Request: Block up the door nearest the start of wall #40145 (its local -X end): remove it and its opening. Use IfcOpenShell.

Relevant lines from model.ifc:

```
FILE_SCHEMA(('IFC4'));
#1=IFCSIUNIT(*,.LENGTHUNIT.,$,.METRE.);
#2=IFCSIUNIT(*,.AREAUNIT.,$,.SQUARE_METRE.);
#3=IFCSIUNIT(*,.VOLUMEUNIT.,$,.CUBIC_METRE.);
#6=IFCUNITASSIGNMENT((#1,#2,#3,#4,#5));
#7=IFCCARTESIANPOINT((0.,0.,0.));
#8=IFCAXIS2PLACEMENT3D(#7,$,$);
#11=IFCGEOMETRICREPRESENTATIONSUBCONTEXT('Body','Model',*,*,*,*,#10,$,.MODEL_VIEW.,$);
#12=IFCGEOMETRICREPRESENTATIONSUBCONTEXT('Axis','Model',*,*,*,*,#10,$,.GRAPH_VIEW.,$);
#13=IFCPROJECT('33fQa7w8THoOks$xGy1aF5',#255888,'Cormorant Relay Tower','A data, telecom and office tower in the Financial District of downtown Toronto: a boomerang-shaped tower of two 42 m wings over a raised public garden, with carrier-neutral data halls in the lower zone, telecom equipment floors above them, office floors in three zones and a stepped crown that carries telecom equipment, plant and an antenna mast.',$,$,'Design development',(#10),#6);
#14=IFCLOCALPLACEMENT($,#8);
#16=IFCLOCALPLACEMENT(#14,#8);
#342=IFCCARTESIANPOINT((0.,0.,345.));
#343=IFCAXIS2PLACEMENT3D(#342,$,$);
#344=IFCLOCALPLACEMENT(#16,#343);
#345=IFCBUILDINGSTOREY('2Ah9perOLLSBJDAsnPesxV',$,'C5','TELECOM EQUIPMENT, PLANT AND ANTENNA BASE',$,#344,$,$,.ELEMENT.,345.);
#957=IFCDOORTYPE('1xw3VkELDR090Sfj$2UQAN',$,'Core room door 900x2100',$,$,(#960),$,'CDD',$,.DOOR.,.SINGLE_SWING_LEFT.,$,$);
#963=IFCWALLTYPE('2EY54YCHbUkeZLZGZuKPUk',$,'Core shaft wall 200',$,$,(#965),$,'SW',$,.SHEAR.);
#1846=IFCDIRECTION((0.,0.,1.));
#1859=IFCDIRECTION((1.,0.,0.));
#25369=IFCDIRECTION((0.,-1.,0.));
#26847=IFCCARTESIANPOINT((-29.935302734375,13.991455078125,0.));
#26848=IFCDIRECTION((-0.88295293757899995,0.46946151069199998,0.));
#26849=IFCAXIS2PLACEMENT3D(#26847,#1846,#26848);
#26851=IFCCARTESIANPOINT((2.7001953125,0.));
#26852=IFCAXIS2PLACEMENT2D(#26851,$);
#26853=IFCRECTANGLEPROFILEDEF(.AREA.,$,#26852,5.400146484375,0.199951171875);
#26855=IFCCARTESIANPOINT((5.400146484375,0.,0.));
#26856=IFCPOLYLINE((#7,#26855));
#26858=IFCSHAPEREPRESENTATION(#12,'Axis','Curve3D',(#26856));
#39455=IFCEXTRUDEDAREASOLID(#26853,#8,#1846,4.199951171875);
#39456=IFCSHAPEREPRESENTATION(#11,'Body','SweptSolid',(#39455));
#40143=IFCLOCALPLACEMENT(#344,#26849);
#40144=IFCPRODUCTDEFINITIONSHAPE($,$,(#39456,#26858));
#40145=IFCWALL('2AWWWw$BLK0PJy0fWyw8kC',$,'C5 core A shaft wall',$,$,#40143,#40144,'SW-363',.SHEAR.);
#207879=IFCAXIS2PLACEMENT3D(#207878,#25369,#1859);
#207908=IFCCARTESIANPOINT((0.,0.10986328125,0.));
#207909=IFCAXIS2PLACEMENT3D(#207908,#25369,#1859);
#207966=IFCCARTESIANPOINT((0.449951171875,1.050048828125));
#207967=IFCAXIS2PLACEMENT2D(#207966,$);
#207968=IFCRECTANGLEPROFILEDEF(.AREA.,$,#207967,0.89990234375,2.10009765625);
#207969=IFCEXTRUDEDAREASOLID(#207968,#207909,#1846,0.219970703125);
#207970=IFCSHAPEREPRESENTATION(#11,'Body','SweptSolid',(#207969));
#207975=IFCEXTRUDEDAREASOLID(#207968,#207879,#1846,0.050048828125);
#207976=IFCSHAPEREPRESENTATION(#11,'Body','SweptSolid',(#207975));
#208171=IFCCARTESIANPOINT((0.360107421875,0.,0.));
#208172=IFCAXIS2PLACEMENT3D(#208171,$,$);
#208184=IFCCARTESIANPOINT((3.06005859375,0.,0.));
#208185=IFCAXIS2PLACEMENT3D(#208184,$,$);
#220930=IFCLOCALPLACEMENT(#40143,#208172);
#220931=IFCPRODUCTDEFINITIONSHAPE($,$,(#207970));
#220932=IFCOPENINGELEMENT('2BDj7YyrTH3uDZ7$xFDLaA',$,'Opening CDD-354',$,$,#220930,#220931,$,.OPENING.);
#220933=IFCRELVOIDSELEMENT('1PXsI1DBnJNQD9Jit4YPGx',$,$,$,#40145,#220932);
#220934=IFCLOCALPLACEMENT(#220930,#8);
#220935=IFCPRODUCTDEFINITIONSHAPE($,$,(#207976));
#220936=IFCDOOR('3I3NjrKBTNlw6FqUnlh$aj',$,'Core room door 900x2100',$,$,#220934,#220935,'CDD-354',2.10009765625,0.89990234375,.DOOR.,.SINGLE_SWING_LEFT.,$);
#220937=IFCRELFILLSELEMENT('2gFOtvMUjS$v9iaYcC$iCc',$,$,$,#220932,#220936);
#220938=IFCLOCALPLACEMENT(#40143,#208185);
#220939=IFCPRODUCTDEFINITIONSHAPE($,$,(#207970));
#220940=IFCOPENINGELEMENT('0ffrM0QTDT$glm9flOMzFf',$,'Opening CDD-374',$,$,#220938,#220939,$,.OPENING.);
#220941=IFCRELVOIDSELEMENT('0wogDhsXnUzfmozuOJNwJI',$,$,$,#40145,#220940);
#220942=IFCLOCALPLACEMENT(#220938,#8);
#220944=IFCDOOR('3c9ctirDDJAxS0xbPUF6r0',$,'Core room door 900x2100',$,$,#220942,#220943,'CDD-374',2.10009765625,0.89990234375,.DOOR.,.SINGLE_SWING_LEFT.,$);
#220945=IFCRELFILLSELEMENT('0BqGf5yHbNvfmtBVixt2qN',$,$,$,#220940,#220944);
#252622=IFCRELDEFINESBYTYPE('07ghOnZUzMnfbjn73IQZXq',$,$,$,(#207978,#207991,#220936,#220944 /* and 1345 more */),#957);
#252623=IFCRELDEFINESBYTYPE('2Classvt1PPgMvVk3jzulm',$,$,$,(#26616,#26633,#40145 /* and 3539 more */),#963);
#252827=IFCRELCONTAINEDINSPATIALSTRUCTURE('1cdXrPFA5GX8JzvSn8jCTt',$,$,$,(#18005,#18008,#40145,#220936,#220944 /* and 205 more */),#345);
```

```python
import ifcopenshell
import ifcopenshell.api.feature
import ifcopenshell.api.root
import ifcopenshell.geom
import ifcopenshell.util.shape

model = ifcopenshell.open("model.ifc")
settings = ifcopenshell.geom.settings()


def volume(element):
    """Net volume in cubic metres, openings subtracted."""
    shape = ifcopenshell.geom.create_shape(settings, element)
    return ifcopenshell.util.shape.get_volume(shape.geometry)


door = model.by_guid("3I3NjrKBTNlw6FqUnlh$aj")
opening = door.FillsVoids[0].RelatingOpeningElement
wall = opening.VoidsElements[0].RelatingBuildingElement
before = volume(wall)

ifcopenshell.api.root.remove_product(model, product=door)
ifcopenshell.api.feature.remove_feature(model, feature=opening)

after = volume(wall)

print(f"wall volume {before:.3f} -> {after:.3f} m3")

model.write("model_edited.ifc")
```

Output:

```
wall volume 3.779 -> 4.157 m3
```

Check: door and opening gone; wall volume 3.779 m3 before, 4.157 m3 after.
